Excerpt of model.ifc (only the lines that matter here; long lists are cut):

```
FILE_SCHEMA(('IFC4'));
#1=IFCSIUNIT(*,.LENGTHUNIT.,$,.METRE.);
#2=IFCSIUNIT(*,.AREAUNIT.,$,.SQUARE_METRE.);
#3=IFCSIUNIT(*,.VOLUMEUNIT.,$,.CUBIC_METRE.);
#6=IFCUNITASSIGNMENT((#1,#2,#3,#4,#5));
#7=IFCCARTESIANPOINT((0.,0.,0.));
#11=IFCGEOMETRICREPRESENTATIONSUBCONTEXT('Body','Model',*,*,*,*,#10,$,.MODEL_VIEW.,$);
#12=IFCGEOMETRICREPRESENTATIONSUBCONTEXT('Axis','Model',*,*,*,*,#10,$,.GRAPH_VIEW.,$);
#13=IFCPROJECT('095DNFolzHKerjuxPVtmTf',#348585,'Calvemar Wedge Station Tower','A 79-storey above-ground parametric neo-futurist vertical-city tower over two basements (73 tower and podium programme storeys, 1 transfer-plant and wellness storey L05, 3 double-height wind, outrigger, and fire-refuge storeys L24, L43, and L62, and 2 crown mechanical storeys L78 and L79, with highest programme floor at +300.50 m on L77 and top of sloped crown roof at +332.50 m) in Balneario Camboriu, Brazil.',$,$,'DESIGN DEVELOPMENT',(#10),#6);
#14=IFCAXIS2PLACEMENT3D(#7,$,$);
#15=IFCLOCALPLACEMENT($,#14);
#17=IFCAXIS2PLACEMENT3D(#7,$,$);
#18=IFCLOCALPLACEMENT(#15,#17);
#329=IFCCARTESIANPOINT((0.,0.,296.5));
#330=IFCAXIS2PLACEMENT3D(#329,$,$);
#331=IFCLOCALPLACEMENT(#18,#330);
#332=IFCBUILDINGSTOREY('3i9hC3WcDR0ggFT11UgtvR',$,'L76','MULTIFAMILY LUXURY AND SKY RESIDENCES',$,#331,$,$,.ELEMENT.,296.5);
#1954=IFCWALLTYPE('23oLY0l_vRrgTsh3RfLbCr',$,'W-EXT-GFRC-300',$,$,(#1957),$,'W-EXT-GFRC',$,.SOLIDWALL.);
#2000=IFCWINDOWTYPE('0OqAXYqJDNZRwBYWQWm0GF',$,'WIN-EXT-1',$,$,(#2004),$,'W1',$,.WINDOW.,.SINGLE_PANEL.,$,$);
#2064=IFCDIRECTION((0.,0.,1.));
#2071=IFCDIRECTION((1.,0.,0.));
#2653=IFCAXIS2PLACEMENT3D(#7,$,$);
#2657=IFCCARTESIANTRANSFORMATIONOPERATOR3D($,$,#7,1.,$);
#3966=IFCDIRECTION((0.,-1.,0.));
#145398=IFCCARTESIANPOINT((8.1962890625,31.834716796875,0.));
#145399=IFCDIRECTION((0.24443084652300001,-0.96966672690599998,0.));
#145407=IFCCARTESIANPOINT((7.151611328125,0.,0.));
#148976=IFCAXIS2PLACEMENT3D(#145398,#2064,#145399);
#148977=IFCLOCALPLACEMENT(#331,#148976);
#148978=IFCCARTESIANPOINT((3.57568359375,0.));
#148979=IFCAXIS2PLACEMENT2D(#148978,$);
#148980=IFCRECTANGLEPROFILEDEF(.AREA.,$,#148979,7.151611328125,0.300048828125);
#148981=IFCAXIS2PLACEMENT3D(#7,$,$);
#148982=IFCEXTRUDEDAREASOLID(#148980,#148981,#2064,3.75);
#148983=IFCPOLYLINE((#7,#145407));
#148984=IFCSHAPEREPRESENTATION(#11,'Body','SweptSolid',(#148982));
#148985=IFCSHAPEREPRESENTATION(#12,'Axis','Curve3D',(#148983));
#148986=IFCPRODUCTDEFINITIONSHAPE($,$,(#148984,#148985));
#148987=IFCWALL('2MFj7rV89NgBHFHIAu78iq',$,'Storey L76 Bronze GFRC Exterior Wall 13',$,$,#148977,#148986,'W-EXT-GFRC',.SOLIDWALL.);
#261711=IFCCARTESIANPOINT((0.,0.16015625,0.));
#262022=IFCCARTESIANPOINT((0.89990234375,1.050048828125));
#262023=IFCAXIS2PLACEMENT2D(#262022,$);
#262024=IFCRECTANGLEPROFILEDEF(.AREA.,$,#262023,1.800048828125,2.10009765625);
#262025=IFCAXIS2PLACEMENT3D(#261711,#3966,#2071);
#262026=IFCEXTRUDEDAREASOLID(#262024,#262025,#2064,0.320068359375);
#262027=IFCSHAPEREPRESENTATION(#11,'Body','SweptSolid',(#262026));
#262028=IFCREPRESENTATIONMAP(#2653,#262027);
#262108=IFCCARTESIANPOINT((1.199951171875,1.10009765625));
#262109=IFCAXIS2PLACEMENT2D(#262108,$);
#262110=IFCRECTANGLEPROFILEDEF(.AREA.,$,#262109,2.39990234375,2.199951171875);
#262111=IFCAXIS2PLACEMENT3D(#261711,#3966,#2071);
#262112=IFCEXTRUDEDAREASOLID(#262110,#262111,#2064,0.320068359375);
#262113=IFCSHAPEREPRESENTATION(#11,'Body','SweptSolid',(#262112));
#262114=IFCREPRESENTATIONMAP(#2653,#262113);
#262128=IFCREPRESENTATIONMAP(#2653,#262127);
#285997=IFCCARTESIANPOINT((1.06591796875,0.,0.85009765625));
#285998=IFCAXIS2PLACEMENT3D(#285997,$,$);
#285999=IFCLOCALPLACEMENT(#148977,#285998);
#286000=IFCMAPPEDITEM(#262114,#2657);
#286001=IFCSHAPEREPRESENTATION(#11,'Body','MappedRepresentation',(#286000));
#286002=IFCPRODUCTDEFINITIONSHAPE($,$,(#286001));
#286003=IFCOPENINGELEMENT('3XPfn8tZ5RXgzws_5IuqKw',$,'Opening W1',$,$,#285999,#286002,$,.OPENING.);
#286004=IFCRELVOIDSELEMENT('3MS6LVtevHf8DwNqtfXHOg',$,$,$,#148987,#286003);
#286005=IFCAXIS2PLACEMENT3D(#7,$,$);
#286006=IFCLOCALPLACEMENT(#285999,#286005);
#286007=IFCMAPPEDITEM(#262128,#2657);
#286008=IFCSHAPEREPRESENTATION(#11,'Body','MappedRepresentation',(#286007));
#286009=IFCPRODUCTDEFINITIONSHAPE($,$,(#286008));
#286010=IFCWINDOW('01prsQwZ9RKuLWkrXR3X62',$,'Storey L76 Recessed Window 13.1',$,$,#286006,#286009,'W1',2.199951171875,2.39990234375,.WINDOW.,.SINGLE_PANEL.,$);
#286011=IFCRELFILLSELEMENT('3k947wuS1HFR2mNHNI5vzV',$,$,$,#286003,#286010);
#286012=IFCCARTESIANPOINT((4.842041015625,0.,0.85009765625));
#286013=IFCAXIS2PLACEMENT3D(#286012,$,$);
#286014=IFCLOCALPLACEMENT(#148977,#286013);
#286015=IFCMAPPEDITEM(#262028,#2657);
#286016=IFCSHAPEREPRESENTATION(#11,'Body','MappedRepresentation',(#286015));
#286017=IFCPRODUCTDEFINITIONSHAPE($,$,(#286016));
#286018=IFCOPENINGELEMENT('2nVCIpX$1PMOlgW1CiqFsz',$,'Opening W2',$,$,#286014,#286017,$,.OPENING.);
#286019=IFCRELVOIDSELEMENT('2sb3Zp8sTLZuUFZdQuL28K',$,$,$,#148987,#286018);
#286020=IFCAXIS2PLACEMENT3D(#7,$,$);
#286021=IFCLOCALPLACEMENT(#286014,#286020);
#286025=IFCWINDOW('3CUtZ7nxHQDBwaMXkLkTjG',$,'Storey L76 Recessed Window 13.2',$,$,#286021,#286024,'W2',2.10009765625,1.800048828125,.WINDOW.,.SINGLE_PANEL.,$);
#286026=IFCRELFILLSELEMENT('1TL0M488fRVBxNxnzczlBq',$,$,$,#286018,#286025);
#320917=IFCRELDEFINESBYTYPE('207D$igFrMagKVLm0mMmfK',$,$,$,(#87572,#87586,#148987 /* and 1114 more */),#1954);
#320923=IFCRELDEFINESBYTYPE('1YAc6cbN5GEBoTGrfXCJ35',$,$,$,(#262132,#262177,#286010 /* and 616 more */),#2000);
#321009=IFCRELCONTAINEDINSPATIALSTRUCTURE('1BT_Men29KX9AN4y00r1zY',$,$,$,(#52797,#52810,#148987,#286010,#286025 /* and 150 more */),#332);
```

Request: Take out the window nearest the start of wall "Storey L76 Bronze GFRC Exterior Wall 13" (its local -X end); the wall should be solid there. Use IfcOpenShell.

```python
import ifcopenshell
import ifcopenshell.api.feature
import ifcopenshell.api.root
import ifcopenshell.geom
import ifcopenshell.util.shape

model = ifcopenshell.open("model.ifc")
settings = ifcopenshell.geom.settings()


def volume(element):
    """Net volume in cubic metres, openings subtracted."""
    shape = ifcopenshell.geom.create_shape(settings, element)
    return ifcopenshell.util.shape.get_volume(shape.geometry)


window = model.by_guid("01prsQwZ9RKuLWkrXR3X62")
opening = window.FillsVoids[0].RelatingOpeningElement
wall = opening.VoidsElements[0].RelatingBuildingElement
before = volume(wall)

ifcopenshell.api.root.remove_product(model, product=window)
ifcopenshell.api.feature.remove_feature(model, feature=opening)

after = volume(wall)

print(f"wall volume {before:.3f} -> {after:.3f} m3")

model.write("model_rev.ifc")
```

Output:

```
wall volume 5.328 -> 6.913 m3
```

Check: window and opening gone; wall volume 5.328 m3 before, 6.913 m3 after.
